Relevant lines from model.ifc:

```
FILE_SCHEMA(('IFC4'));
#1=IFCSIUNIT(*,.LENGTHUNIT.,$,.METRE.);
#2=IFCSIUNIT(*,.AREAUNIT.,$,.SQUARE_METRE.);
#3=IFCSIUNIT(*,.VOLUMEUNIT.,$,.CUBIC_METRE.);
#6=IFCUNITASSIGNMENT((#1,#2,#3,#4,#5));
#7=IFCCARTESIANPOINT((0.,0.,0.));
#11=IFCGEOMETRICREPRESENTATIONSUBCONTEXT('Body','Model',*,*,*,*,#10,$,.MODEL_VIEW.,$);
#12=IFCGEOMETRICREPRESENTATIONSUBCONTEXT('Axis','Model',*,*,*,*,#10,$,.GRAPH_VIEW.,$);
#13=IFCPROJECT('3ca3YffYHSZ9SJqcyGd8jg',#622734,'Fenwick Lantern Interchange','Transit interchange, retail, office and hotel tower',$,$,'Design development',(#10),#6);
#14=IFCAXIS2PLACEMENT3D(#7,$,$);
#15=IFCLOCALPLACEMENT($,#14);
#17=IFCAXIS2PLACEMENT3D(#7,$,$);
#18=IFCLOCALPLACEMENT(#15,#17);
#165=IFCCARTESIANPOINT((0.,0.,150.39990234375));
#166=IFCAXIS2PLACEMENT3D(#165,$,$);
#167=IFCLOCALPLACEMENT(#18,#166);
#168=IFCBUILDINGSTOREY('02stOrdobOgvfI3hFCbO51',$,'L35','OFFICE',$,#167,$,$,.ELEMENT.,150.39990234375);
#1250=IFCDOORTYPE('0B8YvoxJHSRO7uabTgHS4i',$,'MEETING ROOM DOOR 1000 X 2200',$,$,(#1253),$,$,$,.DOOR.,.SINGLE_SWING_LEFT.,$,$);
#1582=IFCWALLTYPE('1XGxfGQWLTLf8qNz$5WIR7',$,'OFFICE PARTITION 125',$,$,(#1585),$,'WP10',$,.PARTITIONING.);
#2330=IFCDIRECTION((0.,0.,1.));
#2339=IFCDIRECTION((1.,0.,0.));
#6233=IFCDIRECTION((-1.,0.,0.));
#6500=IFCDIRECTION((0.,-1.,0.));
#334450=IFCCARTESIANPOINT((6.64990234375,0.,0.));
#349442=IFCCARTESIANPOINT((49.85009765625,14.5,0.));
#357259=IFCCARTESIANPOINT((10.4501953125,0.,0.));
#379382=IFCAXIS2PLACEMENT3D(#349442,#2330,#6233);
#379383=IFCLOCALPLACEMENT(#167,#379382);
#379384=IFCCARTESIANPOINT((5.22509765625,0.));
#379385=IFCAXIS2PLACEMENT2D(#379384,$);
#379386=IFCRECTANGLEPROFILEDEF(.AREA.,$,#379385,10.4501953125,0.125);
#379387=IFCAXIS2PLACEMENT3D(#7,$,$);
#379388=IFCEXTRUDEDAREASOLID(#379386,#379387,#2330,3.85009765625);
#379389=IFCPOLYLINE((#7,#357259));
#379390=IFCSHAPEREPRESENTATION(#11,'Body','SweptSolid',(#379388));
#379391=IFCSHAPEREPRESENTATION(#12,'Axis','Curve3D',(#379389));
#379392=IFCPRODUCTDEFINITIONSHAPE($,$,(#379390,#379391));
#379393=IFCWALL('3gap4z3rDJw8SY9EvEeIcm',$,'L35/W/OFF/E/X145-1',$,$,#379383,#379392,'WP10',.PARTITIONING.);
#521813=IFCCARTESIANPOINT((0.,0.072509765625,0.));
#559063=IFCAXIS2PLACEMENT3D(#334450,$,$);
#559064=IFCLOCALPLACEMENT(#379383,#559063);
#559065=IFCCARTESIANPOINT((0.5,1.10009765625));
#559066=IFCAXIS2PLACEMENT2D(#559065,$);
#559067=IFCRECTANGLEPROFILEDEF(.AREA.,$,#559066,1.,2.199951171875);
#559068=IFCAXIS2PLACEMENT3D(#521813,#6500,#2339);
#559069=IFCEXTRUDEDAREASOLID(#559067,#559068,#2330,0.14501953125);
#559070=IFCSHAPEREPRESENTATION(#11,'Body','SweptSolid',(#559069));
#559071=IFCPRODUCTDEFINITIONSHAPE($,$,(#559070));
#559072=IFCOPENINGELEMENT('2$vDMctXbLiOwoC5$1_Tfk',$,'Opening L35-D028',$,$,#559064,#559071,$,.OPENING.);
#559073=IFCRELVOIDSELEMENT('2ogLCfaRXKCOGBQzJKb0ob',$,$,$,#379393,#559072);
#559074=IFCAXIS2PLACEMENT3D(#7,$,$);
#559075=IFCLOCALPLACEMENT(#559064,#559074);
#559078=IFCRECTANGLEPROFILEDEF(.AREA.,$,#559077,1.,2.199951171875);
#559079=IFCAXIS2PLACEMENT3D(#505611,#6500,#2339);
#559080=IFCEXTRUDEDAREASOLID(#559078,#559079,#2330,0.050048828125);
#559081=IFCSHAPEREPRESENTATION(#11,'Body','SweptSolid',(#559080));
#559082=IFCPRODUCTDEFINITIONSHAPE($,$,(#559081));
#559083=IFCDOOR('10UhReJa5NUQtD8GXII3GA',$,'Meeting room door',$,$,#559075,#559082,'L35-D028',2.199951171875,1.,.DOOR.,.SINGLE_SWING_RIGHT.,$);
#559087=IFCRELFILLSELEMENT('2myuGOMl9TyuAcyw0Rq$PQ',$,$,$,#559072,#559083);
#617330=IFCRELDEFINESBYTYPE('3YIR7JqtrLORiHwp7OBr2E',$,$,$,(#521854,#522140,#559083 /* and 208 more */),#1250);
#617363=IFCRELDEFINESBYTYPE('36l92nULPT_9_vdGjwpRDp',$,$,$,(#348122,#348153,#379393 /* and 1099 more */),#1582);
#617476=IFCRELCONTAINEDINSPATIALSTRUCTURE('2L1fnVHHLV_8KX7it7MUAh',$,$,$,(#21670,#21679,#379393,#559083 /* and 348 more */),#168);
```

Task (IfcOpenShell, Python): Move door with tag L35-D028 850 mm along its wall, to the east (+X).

```python
import ifcopenshell
import ifcopenshell.api.geometry
import ifcopenshell.util.placement
import ifcopenshell.util.unit

model = ifcopenshell.open("model.ifc")
unit_scale = ifcopenshell.util.unit.calculate_unit_scale(model)

door = model.by_guid("10UhReJa5NUQtD8GXII3GA")
opening = door.FillsVoids[0].RelatingOpeningElement
wall = opening.VoidsElements[0].RelatingBuildingElement

wall_matrix = ifcopenshell.util.placement.get_local_placement(wall.ObjectPlacement)
shift = wall_matrix[:3, 0] * -0.85 / unit_scale
before = ifcopenshell.util.placement.get_local_placement(door.ObjectPlacement)[:3, 3].copy()

# The door is placed relative to its opening, so it follows when the opening moves.
matrix = ifcopenshell.util.placement.get_local_placement(opening.ObjectPlacement)
matrix[:3, 3] += shift
ifcopenshell.api.geometry.edit_object_placement(
    model, product=opening, matrix=matrix, is_si=False, should_transform_children=True
)

after = ifcopenshell.util.placement.get_local_placement(door.ObjectPlacement)[:3, 3]
print("door moved by", (after - before).round(3) + 0.0)

model.write("model_rev.ifc")
```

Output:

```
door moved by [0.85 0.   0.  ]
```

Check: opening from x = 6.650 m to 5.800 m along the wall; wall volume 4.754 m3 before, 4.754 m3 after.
